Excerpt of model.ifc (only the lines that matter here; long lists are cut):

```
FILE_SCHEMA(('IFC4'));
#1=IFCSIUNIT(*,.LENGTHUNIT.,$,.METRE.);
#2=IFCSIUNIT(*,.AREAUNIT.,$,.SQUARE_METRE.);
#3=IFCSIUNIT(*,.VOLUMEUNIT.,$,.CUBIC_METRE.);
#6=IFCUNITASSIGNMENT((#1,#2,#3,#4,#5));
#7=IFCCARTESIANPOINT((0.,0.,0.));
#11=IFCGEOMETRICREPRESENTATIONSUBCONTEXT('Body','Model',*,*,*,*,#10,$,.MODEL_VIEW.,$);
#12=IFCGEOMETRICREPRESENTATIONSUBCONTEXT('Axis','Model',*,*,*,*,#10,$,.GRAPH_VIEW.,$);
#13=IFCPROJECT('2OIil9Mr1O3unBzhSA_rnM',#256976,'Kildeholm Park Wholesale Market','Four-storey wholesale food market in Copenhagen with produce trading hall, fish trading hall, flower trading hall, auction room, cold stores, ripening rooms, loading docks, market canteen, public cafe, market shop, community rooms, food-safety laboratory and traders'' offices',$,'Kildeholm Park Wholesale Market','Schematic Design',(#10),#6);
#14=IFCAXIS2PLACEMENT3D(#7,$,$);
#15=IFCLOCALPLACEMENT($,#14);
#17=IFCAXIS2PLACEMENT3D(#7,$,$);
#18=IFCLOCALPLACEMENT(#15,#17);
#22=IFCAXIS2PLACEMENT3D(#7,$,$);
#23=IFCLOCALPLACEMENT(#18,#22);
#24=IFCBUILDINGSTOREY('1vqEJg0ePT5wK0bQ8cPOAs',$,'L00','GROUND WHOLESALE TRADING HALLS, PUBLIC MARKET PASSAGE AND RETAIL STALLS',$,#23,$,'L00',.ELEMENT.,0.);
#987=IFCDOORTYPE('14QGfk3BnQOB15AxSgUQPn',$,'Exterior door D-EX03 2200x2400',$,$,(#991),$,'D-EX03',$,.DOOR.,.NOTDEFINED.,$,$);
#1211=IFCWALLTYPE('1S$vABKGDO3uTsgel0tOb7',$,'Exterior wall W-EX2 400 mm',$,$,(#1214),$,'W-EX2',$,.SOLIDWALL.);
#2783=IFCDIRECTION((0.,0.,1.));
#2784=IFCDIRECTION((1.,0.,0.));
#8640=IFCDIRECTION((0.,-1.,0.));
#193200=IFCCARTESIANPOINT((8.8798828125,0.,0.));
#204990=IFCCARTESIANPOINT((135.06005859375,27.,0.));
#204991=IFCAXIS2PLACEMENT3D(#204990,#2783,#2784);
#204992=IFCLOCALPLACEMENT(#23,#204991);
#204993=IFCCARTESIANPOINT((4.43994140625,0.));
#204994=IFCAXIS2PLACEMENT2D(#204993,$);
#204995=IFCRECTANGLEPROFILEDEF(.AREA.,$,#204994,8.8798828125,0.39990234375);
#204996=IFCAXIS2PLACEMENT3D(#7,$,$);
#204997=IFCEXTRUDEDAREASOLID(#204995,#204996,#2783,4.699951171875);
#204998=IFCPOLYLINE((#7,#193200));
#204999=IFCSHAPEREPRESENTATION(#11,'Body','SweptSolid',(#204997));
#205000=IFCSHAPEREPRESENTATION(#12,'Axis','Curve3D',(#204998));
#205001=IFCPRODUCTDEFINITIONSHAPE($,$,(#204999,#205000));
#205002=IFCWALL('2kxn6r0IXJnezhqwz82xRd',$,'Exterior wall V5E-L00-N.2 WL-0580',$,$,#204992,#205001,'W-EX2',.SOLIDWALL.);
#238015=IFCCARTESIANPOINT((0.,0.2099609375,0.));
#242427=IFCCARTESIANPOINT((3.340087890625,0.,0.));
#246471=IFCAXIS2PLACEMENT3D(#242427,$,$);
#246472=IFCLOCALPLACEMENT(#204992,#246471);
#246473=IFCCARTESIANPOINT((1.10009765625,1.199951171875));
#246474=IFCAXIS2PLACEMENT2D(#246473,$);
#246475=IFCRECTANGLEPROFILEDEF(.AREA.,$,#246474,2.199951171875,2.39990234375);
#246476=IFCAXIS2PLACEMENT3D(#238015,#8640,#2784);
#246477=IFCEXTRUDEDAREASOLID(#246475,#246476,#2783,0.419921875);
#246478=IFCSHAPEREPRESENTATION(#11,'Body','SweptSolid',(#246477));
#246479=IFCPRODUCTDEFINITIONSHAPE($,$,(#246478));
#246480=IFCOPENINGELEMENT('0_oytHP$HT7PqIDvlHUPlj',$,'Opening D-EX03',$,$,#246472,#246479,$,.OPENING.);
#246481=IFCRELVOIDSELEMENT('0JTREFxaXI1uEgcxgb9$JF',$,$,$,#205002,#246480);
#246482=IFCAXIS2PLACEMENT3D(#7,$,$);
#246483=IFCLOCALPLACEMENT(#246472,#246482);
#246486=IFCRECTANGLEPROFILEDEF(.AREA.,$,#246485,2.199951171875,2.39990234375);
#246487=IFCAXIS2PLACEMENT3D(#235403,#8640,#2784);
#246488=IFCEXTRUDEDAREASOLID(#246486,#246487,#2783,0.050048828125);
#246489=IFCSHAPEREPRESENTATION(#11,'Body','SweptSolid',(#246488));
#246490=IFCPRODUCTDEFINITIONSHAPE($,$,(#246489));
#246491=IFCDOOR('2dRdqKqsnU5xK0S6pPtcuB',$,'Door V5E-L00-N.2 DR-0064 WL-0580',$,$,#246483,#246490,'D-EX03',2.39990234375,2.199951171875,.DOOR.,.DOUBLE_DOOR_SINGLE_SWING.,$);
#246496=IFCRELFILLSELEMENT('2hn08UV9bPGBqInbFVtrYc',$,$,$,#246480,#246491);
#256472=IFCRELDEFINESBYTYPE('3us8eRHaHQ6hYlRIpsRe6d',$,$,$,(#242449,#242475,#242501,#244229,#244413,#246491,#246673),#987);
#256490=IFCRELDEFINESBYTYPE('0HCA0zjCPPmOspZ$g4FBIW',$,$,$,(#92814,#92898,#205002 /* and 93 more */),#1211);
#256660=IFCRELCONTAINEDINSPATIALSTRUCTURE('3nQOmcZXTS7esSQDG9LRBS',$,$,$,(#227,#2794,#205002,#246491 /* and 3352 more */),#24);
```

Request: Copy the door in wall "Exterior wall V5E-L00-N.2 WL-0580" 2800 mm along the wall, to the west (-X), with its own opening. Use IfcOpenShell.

```python
import ifcopenshell
import ifcopenshell.api.feature
import ifcopenshell.api.geometry
import ifcopenshell.api.root
import ifcopenshell.geom
import ifcopenshell.util.element
import ifcopenshell.util.placement
import ifcopenshell.util.shape

model = ifcopenshell.open("model.ifc")
settings = ifcopenshell.geom.settings()


def volume(element):
    """Net volume in cubic metres, openings subtracted."""
    shape = ifcopenshell.geom.create_shape(settings, element)
    return ifcopenshell.util.shape.get_volume(shape.geometry)


door = model.by_guid("2dRdqKqsnU5xK0S6pPtcuB")
opening = door.FillsVoids[0].RelatingOpeningElement
wall = opening.VoidsElements[0].RelatingBuildingElement
before = volume(wall)
shift = ifcopenshell.util.placement.get_local_placement(wall.ObjectPlacement)[:3, 0] * -2.8

# copy_class copies the void relationship, type, container and properties, but no geometry.
new_opening = ifcopenshell.api.root.copy_class(model, product=opening)
new_opening.Representation = ifcopenshell.util.element.copy_deep(
    model, opening.Representation, exclude=["IfcGeometricRepresentationContext", "IfcRepresentationMap"]
)
new_door = ifcopenshell.api.root.copy_class(model, product=door)
new_door.Representation = ifcopenshell.util.element.copy_deep(
    model, door.Representation, exclude=["IfcGeometricRepresentationContext", "IfcRepresentationMap"]
)
new_door.Tag = None
ifcopenshell.api.feature.add_filling(model, opening=new_opening, element=new_door)

for old, new in ((opening, new_opening), (door, new_door)):
    matrix = ifcopenshell.util.placement.get_local_placement(old.ObjectPlacement)
    matrix[:3, 3] += shift
    ifcopenshell.api.geometry.edit_object_placement(model, product=new, matrix=matrix, is_si=False)

after = volume(wall)

print(f"wall volume {before:.3f} -> {after:.3f} m3")

model.write("model_edited.ifc")
```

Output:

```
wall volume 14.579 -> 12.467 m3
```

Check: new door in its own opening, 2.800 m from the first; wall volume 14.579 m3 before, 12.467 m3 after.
